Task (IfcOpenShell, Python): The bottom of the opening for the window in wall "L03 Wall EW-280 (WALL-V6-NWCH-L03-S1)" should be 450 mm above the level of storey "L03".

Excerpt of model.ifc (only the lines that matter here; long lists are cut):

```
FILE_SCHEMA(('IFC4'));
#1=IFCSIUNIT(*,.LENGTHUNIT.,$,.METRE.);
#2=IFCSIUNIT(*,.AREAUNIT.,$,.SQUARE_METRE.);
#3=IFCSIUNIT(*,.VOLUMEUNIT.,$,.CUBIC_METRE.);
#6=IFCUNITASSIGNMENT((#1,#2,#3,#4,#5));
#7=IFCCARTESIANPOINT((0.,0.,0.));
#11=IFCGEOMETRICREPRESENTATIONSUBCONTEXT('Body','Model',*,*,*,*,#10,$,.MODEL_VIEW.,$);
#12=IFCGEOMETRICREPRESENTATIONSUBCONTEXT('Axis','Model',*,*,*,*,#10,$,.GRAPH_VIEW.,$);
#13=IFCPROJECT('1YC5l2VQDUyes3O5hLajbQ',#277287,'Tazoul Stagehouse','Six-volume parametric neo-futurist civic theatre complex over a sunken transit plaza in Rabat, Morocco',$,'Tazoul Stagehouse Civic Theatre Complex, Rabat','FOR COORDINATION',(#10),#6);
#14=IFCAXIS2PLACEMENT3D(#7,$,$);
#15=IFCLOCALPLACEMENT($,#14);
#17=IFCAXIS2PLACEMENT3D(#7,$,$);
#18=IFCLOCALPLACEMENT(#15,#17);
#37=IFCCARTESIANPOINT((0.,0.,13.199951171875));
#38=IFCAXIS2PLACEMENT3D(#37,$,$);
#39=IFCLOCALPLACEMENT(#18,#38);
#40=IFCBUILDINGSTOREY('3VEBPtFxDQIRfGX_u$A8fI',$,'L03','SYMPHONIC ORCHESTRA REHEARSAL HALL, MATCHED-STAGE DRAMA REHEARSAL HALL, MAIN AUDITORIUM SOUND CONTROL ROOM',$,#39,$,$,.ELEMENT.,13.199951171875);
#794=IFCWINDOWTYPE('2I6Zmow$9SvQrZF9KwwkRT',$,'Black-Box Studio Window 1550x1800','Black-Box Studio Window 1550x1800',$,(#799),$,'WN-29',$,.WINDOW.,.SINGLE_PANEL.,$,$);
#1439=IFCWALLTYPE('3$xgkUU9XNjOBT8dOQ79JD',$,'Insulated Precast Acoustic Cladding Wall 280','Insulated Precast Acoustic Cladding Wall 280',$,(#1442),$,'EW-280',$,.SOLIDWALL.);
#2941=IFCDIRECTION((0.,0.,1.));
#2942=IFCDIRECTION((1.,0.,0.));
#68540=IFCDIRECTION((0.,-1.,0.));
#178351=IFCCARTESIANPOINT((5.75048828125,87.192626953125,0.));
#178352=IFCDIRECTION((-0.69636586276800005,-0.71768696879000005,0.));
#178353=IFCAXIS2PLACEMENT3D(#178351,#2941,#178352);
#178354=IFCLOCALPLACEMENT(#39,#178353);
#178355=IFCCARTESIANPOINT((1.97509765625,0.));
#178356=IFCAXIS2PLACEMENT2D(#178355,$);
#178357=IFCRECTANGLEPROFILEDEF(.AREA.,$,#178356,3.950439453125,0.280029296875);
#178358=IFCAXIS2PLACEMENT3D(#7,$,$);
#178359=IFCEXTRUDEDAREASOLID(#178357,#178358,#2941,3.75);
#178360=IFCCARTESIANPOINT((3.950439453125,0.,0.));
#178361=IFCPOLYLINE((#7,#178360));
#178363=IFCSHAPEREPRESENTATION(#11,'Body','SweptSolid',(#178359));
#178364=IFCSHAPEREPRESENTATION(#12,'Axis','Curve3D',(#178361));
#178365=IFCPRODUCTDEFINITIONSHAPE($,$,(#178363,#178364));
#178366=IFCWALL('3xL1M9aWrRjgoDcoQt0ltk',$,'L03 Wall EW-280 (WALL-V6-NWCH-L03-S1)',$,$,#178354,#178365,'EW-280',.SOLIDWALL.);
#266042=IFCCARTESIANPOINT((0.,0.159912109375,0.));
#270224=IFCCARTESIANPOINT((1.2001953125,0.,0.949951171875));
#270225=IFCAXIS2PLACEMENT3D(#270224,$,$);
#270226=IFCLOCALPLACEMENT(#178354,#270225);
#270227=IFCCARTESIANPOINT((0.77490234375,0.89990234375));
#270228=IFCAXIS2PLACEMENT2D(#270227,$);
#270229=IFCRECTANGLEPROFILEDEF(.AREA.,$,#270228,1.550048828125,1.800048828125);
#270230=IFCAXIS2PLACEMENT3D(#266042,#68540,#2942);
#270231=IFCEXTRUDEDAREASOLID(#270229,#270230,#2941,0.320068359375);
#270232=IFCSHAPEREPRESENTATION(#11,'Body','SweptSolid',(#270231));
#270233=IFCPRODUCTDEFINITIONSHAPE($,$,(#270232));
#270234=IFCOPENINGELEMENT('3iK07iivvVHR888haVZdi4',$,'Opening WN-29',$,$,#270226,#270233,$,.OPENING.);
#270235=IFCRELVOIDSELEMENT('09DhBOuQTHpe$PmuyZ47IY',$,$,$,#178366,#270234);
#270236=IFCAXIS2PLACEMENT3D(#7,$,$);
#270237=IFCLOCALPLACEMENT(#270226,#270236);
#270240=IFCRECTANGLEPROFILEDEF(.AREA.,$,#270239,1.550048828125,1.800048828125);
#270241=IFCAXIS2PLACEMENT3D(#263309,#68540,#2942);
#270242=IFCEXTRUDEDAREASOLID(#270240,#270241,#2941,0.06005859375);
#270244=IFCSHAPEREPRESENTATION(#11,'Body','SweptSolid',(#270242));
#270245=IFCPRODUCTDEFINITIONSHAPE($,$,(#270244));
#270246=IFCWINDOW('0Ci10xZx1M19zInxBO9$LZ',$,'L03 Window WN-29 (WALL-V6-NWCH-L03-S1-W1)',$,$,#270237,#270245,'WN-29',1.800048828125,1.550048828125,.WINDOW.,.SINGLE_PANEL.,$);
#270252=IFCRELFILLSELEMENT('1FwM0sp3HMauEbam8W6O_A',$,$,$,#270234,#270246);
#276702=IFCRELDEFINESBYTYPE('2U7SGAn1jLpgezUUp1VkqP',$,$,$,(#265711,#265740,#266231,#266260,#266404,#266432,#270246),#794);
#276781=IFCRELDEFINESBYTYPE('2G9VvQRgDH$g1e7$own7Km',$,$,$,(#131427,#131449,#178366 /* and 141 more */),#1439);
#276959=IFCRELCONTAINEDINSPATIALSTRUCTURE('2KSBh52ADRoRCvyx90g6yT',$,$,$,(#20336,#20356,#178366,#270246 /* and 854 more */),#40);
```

```python
import numpy as np
import ifcopenshell
import ifcopenshell.api.geometry
import ifcopenshell.geom
import ifcopenshell.util.element
import ifcopenshell.util.placement
import ifcopenshell.util.shape
import ifcopenshell.util.unit

model = ifcopenshell.open("model.ifc")
unit_scale = ifcopenshell.util.unit.calculate_unit_scale(model)

window = model.by_guid("0Ci10xZx1M19zInxBO9$LZ")
opening = window.FillsVoids[0].RelatingOpeningElement
storey = ifcopenshell.util.element.get_container(window, ifc_class="IfcBuildingStorey")
level = ifcopenshell.util.placement.get_local_placement(storey.ObjectPlacement)[2, 3]

# The opening's origin need not be at the sill, so measure its lowest point.
shape = ifcopenshell.geom.create_shape(ifcopenshell.geom.settings(), opening)
bottom = ifcopenshell.util.shape.get_shape_bottom_elevation(shape, shape.geometry) / unit_scale
dz = level + 0.45 / unit_scale - bottom

shift = np.array([0.0, 0.0, dz])
# The window is placed relative to its opening, so it follows when the opening moves.
matrix = ifcopenshell.util.placement.get_local_placement(opening.ObjectPlacement)
matrix[:3, 3] += shift
ifcopenshell.api.geometry.edit_object_placement(
    model, product=opening, matrix=matrix, is_si=False, should_transform_children=True
)

print(f"moved by {dz * unit_scale:+.3f} m")

model.write("model-out.ifc")
```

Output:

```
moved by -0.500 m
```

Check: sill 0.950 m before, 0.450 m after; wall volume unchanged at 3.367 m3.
